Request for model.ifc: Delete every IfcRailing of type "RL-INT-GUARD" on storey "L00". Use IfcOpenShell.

First a look at what the model holds.

```python
import ifcopenshell
import ifcopenshell.util.element

model = ifcopenshell.open("model.ifc")
print(model.schema)
storey = next(s for s in model.by_type("IfcBuildingStorey") if s.Name == "L00")
railings = [e for e in ifcopenshell.util.element.get_decomposition(storey) if e.is_a("IfcRailing")]
seen = {}
for e in railings:
    element_type = ifcopenshell.util.element.get_type(e)
    name = element_type.Name if element_type not in (None, e) else None
    seen[name] = seen.get(name, 0) + 1
for name, count in sorted(seen.items(), key=str):
    print(count, "x", name)
```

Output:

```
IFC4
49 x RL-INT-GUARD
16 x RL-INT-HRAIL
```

```python
import ifcopenshell
import ifcopenshell.api.root
import ifcopenshell.util.element

model = ifcopenshell.open("model.ifc")

storey = next(s for s in model.by_type("IfcBuildingStorey") if s.Name == "L00")
railings = [e for e in ifcopenshell.util.element.get_decomposition(storey) if e.is_a("IfcRailing")]
targets = [e for e in railings if (t := ifcopenshell.util.element.get_type(e)) not in (None, e) and t.Name == "RL-INT-GUARD"]

for e in targets:
    ifcopenshell.api.root.remove_product(model, product=e)
print(len(targets), "removed")

model.write("model_rev.ifc")
```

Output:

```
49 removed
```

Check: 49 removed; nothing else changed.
